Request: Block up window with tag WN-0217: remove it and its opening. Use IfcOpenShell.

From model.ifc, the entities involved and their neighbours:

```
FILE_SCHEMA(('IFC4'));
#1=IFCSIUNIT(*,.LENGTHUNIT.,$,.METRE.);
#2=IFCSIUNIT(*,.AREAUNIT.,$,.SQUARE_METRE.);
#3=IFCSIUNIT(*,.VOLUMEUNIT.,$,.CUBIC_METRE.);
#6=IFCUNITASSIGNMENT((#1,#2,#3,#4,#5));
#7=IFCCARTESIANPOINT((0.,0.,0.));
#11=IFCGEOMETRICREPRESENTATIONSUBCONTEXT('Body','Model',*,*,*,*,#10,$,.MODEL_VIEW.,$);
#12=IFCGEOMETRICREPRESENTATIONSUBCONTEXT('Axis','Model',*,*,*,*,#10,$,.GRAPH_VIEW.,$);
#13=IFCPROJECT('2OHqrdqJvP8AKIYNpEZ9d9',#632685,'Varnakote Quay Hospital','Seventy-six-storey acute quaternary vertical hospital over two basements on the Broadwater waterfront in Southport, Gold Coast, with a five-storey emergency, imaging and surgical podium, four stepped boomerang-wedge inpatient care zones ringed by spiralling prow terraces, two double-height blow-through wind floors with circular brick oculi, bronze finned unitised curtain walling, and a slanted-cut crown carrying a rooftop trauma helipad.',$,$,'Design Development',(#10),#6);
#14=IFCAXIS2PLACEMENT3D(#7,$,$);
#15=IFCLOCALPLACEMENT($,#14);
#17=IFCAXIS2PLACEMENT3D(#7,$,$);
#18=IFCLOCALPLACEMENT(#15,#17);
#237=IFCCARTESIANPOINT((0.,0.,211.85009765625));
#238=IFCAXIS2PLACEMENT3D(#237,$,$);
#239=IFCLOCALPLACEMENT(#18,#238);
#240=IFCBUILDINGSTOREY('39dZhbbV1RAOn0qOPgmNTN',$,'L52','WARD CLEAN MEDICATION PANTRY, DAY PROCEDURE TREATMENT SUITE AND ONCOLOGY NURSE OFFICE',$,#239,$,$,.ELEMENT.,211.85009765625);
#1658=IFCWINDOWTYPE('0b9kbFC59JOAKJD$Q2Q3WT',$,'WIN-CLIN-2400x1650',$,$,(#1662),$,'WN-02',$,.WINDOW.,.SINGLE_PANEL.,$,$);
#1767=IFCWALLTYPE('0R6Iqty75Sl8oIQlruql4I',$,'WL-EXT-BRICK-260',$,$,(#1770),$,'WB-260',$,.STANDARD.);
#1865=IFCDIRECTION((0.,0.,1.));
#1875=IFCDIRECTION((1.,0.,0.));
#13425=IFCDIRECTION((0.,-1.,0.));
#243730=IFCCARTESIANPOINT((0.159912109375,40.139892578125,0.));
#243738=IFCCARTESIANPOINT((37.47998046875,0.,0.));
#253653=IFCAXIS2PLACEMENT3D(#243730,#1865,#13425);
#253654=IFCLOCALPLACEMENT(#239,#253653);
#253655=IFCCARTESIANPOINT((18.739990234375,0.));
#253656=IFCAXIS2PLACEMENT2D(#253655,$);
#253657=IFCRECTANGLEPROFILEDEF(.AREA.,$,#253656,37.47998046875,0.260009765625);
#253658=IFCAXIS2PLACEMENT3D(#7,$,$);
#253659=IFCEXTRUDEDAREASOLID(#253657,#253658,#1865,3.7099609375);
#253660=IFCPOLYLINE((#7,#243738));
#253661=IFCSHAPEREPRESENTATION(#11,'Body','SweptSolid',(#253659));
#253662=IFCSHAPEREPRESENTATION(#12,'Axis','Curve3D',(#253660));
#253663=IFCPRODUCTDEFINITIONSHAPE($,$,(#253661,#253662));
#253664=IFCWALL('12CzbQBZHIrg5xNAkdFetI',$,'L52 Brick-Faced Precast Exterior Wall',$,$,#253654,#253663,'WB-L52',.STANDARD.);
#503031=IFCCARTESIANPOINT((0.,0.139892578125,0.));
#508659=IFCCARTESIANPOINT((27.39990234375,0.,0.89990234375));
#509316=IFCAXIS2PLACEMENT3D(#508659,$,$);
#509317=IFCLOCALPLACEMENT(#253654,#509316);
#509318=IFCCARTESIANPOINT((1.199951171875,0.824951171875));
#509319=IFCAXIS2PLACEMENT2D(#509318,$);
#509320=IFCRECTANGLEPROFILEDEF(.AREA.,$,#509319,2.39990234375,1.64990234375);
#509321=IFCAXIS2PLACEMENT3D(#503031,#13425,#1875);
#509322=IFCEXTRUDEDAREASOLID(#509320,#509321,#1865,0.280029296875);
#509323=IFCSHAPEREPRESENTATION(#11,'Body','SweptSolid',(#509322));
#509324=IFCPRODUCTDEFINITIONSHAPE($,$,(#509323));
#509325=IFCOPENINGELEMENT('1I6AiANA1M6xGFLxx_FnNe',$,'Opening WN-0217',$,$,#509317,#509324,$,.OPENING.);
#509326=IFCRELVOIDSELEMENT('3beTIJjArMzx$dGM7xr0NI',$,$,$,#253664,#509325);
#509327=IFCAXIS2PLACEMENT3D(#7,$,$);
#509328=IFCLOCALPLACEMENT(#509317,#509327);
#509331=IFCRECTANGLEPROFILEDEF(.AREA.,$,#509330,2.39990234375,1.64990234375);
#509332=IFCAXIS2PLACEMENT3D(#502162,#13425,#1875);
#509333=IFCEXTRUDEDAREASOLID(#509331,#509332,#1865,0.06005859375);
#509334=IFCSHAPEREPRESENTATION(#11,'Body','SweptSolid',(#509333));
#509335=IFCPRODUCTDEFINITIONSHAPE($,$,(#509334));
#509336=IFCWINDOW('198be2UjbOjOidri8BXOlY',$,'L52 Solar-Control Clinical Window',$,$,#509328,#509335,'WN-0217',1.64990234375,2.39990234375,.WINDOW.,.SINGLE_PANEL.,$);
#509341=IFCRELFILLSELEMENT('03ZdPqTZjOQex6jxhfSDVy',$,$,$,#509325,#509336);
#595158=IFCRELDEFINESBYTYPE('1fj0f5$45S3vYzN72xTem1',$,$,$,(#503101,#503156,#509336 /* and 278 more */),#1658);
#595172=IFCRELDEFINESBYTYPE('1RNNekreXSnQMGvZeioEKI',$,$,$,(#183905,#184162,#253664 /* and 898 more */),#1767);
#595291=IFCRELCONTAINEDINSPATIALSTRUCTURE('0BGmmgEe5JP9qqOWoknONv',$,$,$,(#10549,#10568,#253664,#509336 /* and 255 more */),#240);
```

```python
import ifcopenshell
import ifcopenshell.api.feature
import ifcopenshell.api.root
import ifcopenshell.geom
import ifcopenshell.util.shape

model = ifcopenshell.open("model.ifc")
settings = ifcopenshell.geom.settings()


def volume(element):
    """Net volume in cubic metres, openings subtracted."""
    shape = ifcopenshell.geom.create_shape(settings, element)
    return ifcopenshell.util.shape.get_volume(shape.geometry)


window = model.by_guid("198be2UjbOjOidri8BXOlY")
opening = window.FillsVoids[0].RelatingOpeningElement
wall = opening.VoidsElements[0].RelatingBuildingElement
before = volume(wall)

ifcopenshell.api.root.remove_product(model, product=window)
ifcopenshell.api.feature.remove_feature(model, feature=opening)

after = volume(wall)

print(f"wall volume {before:.3f} -> {after:.3f} m3")

model.write("model-out.ifc")
```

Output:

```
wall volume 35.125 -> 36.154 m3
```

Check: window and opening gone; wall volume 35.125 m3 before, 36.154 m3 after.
